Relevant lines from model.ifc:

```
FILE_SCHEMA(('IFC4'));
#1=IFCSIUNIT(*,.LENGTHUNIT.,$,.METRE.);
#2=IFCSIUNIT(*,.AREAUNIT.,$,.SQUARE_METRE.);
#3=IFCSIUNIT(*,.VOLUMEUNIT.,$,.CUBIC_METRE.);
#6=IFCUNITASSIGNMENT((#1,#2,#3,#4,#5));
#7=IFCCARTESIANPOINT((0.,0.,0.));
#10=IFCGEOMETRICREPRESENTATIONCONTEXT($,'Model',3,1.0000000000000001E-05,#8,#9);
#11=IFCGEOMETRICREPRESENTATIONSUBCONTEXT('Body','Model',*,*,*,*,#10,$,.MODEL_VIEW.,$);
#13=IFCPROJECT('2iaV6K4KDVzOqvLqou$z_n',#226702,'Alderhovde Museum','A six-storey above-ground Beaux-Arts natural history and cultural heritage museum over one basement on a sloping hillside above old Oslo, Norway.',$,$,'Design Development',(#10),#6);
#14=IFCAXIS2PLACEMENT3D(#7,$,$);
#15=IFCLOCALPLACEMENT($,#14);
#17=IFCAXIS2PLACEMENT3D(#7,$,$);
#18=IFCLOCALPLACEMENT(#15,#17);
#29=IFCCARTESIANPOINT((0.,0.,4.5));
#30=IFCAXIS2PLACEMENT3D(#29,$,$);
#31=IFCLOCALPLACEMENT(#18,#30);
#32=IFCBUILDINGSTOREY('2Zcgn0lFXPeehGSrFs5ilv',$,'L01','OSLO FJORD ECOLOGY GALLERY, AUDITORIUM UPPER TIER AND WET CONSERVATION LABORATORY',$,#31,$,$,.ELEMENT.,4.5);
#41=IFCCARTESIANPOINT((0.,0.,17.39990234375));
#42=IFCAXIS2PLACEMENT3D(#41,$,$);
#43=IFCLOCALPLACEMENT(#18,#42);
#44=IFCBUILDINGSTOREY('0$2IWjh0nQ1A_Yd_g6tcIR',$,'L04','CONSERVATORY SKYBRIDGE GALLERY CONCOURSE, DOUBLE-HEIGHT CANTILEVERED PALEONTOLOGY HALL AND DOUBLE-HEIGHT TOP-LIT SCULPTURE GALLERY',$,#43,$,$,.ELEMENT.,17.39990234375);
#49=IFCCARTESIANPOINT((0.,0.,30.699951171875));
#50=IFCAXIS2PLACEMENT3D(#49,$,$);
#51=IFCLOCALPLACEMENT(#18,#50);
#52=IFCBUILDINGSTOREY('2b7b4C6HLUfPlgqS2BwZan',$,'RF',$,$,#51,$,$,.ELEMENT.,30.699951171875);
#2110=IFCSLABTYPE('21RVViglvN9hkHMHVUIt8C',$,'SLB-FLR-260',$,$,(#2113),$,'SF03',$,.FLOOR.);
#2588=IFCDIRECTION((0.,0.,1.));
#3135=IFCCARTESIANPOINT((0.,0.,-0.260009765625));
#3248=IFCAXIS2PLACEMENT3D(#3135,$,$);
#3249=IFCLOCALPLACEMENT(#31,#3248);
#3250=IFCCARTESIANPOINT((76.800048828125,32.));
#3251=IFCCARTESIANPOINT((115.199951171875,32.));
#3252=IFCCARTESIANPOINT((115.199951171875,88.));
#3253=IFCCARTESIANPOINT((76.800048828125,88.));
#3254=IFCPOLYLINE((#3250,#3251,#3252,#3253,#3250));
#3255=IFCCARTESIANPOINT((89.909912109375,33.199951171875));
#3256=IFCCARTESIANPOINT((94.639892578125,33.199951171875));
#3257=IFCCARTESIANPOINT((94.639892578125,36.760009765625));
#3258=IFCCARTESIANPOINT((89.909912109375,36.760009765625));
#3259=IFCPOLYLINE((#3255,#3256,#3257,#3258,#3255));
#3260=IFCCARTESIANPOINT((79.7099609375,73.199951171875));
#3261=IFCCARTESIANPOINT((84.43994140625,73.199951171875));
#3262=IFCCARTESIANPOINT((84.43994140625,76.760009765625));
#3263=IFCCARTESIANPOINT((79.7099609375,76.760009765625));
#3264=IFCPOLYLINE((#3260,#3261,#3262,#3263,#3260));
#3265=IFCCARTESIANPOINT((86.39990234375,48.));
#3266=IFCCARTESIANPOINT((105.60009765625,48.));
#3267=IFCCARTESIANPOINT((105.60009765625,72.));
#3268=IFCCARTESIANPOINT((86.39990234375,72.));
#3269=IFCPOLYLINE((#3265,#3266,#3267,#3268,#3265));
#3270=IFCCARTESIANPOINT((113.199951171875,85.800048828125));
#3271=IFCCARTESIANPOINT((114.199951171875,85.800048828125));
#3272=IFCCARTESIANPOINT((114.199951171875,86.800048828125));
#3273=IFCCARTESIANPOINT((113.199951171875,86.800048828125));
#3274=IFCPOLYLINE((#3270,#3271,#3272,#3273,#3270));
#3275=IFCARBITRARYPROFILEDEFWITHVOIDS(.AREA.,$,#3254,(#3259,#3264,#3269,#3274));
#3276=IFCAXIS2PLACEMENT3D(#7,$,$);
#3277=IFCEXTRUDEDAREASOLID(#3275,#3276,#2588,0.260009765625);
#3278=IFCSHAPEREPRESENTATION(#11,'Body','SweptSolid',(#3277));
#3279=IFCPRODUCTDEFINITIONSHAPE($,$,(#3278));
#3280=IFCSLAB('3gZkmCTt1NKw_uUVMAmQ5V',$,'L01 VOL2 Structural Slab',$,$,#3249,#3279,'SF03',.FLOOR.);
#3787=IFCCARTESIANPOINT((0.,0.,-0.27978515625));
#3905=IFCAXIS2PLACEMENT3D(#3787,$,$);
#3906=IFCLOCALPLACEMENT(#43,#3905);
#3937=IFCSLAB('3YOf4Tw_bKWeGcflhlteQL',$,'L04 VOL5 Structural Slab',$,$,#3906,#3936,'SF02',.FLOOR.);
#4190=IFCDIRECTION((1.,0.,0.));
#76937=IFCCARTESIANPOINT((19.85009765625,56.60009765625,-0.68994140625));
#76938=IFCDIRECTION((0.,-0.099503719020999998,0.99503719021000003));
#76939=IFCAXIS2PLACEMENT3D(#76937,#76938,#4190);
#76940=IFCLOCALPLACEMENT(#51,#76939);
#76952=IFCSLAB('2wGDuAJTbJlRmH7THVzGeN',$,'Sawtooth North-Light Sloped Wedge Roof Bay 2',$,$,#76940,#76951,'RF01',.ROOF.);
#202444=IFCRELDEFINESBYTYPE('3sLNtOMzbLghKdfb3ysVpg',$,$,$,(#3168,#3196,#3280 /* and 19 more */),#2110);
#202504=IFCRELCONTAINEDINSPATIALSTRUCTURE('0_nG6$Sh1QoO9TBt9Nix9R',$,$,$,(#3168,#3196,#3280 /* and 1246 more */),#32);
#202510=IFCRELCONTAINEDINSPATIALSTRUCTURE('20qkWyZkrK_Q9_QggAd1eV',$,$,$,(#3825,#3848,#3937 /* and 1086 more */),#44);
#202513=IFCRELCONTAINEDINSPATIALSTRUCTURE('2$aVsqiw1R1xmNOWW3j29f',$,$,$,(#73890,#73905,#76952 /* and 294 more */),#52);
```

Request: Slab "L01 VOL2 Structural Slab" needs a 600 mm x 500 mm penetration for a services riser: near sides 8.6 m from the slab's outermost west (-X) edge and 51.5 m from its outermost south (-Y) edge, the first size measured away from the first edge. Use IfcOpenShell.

```python
import numpy as np
import ifcopenshell
import ifcopenshell.api.feature
import ifcopenshell.api.geometry
import ifcopenshell.api.root
import ifcopenshell.geom
import ifcopenshell.util.placement
import ifcopenshell.util.representation
import ifcopenshell.util.shape
import ifcopenshell.util.unit

model = ifcopenshell.open("model.ifc")
unit_scale = ifcopenshell.util.unit.calculate_unit_scale(model)
settings = ifcopenshell.geom.settings()


def volume(element):
    """Net volume in cubic metres, openings subtracted."""
    shape = ifcopenshell.geom.create_shape(settings, element)
    return ifcopenshell.util.shape.get_volume(shape.geometry)


slab = model.by_id(3280)
before = volume(slab)

# Extent in the slab's own axes, in metres. The edges named are its -X and -Y sides.
slab_shape = ifcopenshell.geom.create_shape(settings, slab)
vertices = ifcopenshell.util.shape.get_vertices(slab_shape.geometry)
x_min, y_min, bottom = vertices.min(axis=0)
top = vertices[:, 2].max()

opening = ifcopenshell.api.root.create_entity(model, ifc_class="IfcOpeningElement", name="Services riser opening", predefined_type="OPENING")
context = ifcopenshell.util.representation.get_context(model, "Model", "Body", "MODEL_VIEW")
width, depth = 0.6, 0.5
outline = [(0.0, 0.0), (width, 0.0), (width, depth), (0.0, depth), (0.0, 0.0)]
# Overshoot both faces by 50 mm so the cut is clean.
shape = ifcopenshell.api.geometry.add_slab_representation(
    model, context=context, depth=top - bottom + 0.1, polyline=outline
)
ifcopenshell.api.geometry.assign_representation(model, product=opening, representation=shape)

matrix = ifcopenshell.util.placement.get_local_placement(slab.ObjectPlacement)
matrix[:, 3] = matrix @ np.append(np.array([x_min + 8.6, y_min + 51.5, bottom - 0.05]) / unit_scale, 1.0)
ifcopenshell.api.geometry.edit_object_placement(model, product=opening, matrix=matrix, is_si=False)
ifcopenshell.api.feature.add_feature(model, feature=opening, element=slab)

after = volume(slab)

print(f"slab volume {before:.3f} -> {after:.3f} m3")

model.write("model_edited.ifc")
```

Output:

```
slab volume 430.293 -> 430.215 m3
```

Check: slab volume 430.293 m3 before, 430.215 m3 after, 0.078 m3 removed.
